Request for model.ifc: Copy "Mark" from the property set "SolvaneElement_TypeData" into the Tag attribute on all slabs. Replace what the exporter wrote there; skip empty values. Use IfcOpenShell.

First a look at what the model holds.

```python
import ifcopenshell
import ifcopenshell.util.element

model = ifcopenshell.open("model.ifc")
print(model.schema)
slabs = model.by_type("IfcSlab")
print(len(slabs), "slabs")
for e in slabs[:8]:
    source = ifcopenshell.util.element.get_pset(e, "SolvaneElement_TypeData", "Mark")
    target = e.Tag
    print(e.id(), repr(source), repr(target), sep=" | ")
```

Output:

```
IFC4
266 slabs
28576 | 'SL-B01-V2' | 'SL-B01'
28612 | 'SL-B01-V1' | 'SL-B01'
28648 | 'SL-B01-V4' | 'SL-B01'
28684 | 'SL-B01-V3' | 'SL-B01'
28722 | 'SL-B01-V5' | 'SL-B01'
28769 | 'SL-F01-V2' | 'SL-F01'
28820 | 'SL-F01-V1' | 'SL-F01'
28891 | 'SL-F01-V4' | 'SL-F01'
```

```python
import ifcopenshell
import ifcopenshell.util.element

model = ifcopenshell.open("model.ifc")

count = 0
for e in model.by_type("IfcSlab"):
    value = ifcopenshell.util.element.get_pset(e, "SolvaneElement_TypeData", "Mark")
    current = e.Tag
    if not value or not value.strip() or current == value:
        continue
    e.Tag = value
    count += 1

print(count, "slabs updated")

model.write("model_rev.ifc")
```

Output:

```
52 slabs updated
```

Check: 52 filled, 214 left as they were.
